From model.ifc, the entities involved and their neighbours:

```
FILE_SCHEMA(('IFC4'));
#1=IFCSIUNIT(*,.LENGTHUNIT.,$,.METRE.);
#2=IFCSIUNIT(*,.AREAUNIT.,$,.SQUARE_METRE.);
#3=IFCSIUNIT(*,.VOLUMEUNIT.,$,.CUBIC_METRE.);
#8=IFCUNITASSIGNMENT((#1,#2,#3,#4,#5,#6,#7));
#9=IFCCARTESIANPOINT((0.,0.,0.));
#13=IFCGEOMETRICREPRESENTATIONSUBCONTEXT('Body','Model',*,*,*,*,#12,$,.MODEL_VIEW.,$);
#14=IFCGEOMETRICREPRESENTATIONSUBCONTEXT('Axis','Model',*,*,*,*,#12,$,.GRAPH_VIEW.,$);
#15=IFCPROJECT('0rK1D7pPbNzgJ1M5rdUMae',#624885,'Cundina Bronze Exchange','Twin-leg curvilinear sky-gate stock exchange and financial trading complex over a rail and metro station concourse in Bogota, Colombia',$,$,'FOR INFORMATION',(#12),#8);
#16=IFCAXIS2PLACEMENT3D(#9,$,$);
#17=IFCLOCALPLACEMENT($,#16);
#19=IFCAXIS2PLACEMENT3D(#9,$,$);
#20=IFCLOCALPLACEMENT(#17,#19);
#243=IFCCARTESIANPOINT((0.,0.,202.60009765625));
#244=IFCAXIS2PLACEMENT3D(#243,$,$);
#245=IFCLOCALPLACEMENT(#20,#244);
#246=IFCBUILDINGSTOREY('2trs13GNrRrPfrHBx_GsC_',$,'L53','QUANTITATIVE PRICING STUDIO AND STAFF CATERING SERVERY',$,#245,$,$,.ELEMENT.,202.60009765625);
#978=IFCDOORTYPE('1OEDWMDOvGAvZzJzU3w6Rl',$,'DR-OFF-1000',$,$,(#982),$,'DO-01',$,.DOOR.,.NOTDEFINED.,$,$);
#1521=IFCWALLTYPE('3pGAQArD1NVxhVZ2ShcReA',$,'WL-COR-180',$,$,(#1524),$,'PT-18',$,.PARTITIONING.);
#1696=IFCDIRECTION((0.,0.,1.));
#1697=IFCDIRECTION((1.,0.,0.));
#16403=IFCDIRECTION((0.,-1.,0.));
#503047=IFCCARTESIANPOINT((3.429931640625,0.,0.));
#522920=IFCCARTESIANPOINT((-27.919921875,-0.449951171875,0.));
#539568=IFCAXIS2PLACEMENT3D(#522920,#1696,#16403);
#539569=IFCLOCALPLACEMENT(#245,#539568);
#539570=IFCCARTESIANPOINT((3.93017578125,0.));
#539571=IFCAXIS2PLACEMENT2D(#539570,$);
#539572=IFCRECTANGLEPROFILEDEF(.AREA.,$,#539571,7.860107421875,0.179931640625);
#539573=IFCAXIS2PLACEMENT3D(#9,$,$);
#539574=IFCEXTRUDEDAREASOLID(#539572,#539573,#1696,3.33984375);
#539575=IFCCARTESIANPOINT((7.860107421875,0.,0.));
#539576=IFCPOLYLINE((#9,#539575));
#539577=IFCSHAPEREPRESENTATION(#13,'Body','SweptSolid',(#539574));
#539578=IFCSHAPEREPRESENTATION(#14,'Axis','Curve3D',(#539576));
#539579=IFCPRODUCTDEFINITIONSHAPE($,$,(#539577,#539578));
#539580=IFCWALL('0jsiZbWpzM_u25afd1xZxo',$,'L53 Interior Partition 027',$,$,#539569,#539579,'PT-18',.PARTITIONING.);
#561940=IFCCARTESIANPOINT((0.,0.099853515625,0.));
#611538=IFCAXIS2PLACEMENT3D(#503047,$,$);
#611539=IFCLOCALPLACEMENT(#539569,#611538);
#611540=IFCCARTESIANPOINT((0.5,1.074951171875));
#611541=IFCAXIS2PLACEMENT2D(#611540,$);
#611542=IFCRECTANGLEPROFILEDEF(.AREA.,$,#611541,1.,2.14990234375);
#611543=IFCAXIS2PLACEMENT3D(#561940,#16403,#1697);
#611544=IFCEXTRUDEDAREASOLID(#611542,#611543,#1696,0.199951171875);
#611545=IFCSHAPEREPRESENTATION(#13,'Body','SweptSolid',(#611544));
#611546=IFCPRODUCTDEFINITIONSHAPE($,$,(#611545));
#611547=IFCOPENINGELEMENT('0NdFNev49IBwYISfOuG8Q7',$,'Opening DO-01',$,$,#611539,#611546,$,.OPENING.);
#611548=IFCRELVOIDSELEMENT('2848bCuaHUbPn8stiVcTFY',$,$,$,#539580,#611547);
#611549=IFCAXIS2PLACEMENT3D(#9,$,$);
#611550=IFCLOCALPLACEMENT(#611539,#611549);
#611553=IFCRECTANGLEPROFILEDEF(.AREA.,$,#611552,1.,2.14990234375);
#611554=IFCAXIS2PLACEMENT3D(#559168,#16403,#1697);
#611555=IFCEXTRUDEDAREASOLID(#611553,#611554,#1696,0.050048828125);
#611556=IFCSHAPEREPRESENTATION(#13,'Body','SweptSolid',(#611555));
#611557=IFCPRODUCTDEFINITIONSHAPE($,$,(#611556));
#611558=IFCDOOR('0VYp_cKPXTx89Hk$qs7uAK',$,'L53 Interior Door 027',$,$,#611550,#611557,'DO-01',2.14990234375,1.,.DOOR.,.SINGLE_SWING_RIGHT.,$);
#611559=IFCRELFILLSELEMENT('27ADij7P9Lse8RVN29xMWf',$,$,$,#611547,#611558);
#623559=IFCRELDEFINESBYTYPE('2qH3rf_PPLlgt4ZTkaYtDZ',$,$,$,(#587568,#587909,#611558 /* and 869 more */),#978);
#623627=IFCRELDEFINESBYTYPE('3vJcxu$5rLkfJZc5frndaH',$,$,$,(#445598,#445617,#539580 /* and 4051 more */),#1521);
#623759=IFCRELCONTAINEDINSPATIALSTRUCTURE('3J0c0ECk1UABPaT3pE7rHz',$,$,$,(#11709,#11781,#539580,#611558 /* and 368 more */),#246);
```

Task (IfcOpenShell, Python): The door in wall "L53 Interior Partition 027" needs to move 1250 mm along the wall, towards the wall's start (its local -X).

```python
import ifcopenshell
import ifcopenshell.api.geometry
import ifcopenshell.util.placement

model = ifcopenshell.open("model.ifc")

door = model.by_guid("0VYp_cKPXTx89Hk$qs7uAK")
opening = door.FillsVoids[0].RelatingOpeningElement
wall = opening.VoidsElements[0].RelatingBuildingElement

wall_matrix = ifcopenshell.util.placement.get_local_placement(wall.ObjectPlacement)
shift = wall_matrix[:3, 0] * -1.25
before = ifcopenshell.util.placement.get_local_placement(door.ObjectPlacement)[:3, 3].copy()

# The door is placed relative to its opening, so it follows when the opening moves.
matrix = ifcopenshell.util.placement.get_local_placement(opening.ObjectPlacement)
matrix[:3, 3] += shift
ifcopenshell.api.geometry.edit_object_placement(
    model, product=opening, matrix=matrix, is_si=False, should_transform_children=True
)

after = ifcopenshell.util.placement.get_local_placement(door.ObjectPlacement)[:3, 3]
print("door moved by", (after - before).round(3) + 0.0)

model.write("model_v2.ifc")
```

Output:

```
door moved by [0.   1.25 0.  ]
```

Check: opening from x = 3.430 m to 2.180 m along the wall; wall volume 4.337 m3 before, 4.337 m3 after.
